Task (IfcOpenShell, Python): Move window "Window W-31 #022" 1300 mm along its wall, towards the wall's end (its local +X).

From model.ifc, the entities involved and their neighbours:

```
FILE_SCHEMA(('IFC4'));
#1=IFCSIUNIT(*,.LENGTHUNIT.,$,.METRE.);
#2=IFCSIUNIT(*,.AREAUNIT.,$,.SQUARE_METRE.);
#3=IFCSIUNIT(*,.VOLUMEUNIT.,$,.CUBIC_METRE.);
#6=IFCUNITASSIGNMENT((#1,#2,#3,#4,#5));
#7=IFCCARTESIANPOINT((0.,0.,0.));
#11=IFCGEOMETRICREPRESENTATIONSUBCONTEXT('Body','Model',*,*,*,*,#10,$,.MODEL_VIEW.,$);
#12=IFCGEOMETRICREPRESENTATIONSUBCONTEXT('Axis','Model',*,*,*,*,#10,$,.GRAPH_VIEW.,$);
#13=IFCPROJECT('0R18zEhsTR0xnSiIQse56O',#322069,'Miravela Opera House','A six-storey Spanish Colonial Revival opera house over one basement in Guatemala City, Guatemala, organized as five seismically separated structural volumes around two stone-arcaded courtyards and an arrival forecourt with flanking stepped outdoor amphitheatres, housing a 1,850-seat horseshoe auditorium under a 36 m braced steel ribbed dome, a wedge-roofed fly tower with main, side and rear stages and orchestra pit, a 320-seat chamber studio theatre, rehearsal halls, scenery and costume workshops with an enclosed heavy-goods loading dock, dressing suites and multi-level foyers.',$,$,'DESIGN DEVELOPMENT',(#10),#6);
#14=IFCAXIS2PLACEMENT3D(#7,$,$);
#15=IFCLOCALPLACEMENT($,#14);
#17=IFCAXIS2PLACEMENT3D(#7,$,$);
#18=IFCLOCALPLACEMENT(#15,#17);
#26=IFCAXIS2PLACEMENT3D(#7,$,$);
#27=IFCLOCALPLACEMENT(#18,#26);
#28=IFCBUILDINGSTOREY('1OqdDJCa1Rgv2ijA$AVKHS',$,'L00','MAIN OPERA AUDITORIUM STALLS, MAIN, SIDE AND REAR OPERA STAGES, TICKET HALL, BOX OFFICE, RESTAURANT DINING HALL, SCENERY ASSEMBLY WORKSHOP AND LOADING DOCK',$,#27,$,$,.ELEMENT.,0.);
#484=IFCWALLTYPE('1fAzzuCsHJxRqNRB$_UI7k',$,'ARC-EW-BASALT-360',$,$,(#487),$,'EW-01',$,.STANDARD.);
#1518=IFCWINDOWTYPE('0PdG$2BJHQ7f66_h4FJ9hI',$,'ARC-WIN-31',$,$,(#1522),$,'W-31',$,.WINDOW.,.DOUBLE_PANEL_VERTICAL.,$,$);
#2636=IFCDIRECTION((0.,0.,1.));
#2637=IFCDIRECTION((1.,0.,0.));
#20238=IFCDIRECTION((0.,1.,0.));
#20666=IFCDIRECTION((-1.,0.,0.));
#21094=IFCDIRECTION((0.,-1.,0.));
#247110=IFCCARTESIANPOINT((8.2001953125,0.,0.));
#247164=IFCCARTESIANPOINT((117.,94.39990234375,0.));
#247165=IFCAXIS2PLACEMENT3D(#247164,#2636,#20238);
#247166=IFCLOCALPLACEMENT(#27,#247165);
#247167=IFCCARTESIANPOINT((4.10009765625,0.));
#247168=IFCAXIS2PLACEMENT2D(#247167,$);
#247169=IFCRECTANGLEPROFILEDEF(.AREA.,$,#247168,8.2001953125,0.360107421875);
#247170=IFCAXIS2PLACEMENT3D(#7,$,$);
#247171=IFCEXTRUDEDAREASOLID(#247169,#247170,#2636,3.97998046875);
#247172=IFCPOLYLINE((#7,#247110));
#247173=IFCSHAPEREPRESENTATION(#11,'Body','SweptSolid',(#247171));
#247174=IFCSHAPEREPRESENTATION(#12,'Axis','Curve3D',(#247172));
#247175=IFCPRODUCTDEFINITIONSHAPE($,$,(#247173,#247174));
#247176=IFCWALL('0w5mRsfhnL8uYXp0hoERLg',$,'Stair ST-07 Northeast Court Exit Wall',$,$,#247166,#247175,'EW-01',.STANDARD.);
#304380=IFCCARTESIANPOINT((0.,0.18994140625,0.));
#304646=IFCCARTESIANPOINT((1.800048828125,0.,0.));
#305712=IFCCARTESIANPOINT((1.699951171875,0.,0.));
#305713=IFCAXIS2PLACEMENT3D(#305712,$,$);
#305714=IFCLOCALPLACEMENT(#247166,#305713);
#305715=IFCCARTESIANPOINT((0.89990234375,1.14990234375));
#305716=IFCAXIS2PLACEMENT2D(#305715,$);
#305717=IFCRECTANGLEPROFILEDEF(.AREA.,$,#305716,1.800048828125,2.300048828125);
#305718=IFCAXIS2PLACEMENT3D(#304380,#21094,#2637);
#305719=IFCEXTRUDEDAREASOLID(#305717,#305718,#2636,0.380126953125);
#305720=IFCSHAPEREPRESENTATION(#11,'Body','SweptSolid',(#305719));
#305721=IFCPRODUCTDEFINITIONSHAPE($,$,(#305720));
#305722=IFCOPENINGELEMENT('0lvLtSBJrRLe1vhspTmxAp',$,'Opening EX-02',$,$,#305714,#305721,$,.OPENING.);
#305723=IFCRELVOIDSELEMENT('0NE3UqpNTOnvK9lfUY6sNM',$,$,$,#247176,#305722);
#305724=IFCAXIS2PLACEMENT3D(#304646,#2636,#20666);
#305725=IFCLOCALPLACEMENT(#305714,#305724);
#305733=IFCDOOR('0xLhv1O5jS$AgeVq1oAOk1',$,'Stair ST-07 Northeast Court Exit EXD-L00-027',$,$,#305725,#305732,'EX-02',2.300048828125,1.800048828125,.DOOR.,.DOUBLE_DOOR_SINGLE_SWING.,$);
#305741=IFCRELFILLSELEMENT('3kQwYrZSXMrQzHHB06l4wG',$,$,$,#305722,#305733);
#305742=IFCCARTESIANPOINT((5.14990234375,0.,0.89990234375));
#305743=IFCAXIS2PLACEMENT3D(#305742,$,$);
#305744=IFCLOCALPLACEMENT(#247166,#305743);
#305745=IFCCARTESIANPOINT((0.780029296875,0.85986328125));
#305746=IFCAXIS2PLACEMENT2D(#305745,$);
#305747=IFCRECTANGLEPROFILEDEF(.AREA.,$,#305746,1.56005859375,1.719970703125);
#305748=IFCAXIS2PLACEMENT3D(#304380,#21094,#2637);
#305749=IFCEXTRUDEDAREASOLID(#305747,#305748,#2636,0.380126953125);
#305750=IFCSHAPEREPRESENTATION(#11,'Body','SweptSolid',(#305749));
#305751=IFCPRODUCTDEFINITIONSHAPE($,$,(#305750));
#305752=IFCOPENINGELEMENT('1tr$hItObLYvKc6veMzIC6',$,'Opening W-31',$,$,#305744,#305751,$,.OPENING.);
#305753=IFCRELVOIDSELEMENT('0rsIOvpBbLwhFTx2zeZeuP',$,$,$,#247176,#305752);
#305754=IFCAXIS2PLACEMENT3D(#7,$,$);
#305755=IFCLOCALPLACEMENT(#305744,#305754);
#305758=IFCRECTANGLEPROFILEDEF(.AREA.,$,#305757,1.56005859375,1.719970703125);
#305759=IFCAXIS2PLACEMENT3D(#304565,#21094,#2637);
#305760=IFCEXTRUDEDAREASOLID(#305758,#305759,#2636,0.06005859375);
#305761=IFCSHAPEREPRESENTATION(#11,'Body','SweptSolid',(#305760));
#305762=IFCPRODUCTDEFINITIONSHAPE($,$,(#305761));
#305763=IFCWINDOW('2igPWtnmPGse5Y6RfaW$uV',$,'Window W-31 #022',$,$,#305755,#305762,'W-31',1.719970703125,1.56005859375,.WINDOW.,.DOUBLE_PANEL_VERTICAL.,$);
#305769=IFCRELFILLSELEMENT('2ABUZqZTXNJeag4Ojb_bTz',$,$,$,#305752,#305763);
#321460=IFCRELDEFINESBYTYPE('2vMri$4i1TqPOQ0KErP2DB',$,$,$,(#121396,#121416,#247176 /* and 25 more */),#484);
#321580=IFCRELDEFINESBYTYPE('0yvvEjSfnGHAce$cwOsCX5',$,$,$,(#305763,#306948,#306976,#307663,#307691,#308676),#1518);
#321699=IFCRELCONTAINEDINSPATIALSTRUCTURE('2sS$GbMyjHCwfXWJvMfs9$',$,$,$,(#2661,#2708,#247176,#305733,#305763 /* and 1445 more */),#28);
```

```python
import ifcopenshell
import ifcopenshell.api.geometry
import ifcopenshell.util.placement
import ifcopenshell.util.unit

model = ifcopenshell.open("model.ifc")
unit_scale = ifcopenshell.util.unit.calculate_unit_scale(model)

window = model.by_guid("2igPWtnmPGse5Y6RfaW$uV")
opening = window.FillsVoids[0].RelatingOpeningElement
wall = opening.VoidsElements[0].RelatingBuildingElement

wall_matrix = ifcopenshell.util.placement.get_local_placement(wall.ObjectPlacement)
shift = wall_matrix[:3, 0] * 1.3 / unit_scale
before = ifcopenshell.util.placement.get_local_placement(window.ObjectPlacement)[:3, 3].copy()

# The window is placed relative to its opening, so it follows when the opening moves.
matrix = ifcopenshell.util.placement.get_local_placement(opening.ObjectPlacement)
matrix[:3, 3] += shift
ifcopenshell.api.geometry.edit_object_placement(
    model, product=opening, matrix=matrix, is_si=False, should_transform_children=True
)

after = ifcopenshell.util.placement.get_local_placement(window.ObjectPlacement)[:3, 3]
print("window moved by", (after - before).round(3) + 0.0)

model.write("model_v2.ifc")
```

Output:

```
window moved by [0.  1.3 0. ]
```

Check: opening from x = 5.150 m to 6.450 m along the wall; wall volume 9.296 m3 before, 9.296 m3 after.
